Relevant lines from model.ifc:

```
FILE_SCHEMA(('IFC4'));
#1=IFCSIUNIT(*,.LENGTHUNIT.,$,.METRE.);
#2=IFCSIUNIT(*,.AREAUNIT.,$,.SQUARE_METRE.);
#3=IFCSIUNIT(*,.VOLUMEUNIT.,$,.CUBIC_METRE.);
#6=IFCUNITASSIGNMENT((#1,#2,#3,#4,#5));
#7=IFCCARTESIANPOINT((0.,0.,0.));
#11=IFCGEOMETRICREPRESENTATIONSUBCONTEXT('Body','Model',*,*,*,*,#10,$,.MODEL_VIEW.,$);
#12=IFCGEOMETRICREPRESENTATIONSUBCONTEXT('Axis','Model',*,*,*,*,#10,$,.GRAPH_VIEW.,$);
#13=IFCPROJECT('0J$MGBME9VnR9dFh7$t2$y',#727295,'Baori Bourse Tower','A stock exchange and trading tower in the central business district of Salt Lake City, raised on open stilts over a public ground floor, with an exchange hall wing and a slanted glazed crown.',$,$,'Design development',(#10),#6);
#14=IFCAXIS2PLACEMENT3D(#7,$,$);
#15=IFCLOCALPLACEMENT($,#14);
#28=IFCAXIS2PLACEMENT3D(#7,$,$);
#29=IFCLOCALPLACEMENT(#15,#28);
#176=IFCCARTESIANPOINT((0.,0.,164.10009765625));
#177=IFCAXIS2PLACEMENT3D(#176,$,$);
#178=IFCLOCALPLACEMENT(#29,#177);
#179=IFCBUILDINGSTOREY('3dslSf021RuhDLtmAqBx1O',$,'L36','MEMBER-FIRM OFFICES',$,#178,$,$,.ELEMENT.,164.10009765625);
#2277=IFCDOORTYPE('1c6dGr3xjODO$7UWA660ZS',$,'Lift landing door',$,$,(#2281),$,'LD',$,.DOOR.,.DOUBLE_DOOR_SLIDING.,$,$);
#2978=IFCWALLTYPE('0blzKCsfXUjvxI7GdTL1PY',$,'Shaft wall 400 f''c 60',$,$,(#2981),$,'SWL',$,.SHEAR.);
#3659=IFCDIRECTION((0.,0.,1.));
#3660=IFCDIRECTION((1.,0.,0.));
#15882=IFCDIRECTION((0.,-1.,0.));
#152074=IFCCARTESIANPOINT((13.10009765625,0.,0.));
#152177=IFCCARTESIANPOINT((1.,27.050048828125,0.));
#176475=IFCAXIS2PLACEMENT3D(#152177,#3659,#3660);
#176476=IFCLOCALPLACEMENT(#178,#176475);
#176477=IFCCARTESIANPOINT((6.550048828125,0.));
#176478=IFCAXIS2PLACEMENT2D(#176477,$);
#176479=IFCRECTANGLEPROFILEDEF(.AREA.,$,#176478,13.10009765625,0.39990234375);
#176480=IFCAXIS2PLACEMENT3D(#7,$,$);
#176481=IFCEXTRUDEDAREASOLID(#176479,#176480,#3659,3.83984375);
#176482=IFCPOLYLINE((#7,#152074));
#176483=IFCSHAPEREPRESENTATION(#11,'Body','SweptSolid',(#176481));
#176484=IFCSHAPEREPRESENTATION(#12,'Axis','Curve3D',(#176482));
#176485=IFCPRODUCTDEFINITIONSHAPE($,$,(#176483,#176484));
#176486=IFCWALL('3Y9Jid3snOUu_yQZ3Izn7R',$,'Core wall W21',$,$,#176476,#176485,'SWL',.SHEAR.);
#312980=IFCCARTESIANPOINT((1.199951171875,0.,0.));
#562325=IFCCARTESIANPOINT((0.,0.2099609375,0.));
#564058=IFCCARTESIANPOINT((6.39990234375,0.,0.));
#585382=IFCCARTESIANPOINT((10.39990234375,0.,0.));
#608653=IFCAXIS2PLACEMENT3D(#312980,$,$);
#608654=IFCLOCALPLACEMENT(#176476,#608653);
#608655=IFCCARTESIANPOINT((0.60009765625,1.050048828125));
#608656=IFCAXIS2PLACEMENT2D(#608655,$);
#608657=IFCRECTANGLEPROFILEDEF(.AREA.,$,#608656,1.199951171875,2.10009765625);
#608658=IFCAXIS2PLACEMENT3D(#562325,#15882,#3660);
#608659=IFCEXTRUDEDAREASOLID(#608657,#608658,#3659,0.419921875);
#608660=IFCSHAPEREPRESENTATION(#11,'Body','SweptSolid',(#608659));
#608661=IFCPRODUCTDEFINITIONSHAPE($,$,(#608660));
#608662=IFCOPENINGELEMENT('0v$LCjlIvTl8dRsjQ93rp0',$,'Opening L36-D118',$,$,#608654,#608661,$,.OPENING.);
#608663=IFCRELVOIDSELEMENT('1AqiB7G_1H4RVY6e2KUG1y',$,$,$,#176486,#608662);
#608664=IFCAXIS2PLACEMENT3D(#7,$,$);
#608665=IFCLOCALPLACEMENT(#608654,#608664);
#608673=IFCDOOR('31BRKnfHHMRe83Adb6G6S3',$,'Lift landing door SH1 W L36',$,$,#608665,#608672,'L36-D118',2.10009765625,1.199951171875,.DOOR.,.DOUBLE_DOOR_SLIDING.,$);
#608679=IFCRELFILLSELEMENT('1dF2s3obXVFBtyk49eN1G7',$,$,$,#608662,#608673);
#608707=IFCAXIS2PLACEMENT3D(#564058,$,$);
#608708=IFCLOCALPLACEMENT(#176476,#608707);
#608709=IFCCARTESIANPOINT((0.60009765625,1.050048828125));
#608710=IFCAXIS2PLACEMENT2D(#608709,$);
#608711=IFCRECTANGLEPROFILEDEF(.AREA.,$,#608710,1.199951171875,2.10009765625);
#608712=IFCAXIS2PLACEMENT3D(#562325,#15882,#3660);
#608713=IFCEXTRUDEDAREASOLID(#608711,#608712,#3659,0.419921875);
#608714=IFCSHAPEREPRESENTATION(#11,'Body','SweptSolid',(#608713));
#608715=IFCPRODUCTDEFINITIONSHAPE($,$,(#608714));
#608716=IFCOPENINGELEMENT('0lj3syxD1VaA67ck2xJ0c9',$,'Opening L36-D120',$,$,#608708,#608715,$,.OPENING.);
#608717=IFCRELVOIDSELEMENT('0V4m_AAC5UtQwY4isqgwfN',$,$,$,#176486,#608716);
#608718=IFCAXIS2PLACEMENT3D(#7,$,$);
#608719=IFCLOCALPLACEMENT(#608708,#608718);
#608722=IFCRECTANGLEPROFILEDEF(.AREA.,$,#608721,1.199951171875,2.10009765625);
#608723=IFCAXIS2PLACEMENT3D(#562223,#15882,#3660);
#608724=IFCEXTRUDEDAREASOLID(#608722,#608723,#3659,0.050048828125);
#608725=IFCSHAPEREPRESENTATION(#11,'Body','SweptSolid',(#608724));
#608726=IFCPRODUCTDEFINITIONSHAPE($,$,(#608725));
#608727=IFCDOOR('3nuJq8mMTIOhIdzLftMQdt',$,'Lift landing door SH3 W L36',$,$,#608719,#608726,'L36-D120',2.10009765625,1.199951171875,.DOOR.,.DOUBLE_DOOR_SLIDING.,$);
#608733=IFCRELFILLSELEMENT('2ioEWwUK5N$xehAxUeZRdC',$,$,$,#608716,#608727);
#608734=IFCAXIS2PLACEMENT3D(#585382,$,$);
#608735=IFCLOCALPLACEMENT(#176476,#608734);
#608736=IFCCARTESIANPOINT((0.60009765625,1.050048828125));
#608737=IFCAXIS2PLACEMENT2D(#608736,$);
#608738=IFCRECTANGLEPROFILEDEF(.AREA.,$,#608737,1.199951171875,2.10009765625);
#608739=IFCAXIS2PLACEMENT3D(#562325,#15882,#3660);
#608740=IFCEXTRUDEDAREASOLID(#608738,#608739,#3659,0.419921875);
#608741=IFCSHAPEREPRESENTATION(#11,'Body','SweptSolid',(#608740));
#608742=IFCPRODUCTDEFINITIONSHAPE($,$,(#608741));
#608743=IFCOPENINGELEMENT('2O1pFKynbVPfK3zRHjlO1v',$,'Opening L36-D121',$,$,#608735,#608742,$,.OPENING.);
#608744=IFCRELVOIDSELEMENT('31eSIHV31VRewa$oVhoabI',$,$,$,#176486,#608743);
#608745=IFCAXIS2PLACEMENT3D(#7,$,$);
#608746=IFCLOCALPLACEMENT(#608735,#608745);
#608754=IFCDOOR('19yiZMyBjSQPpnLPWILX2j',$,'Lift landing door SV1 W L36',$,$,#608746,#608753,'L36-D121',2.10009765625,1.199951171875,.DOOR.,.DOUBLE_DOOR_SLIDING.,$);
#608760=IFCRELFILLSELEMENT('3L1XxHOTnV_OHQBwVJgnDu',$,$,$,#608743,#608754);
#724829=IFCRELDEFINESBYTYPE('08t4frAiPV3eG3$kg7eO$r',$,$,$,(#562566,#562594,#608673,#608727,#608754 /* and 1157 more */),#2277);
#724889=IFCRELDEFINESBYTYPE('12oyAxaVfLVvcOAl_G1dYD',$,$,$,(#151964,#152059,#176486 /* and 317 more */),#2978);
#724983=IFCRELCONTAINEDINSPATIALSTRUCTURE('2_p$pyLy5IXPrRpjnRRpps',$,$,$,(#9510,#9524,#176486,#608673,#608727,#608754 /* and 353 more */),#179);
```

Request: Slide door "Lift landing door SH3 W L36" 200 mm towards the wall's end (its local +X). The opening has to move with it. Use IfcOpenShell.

```python
import ifcopenshell
import ifcopenshell.api.geometry
import ifcopenshell.util.placement

model = ifcopenshell.open("model.ifc")

door = model.by_id(608727)
opening = door.FillsVoids[0].RelatingOpeningElement
wall = opening.VoidsElements[0].RelatingBuildingElement

wall_matrix = ifcopenshell.util.placement.get_local_placement(wall.ObjectPlacement)
shift = wall_matrix[:3, 0] * 0.2
before = ifcopenshell.util.placement.get_local_placement(door.ObjectPlacement)[:3, 3].copy()

# The door is placed relative to its opening, so it follows when the opening moves.
matrix = ifcopenshell.util.placement.get_local_placement(opening.ObjectPlacement)
matrix[:3, 3] += shift
ifcopenshell.api.geometry.edit_object_placement(
    model, product=opening, matrix=matrix, is_si=False, should_transform_children=True
)

after = ifcopenshell.util.placement.get_local_placement(door.ObjectPlacement)[:3, 3]
print("door moved by", (after - before).round(3) + 0.0)

model.write("model_rev.ifc")
```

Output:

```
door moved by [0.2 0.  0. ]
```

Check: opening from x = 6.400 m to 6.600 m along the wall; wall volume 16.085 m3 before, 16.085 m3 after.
